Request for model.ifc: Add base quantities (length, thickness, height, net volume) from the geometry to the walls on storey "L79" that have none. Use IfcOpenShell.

First a look at what the model holds.

```python
import ifcopenshell
import ifcopenshell.util.element
import ifcopenshell.util.unit

model = ifcopenshell.open("model.ifc")
print(model.schema)
for unit_type in ("LENGTHUNIT", "AREAUNIT", "VOLUMEUNIT"):
    print(unit_type, ifcopenshell.util.unit.calculate_unit_scale(model, unit_type))
storey = next(s for s in model.by_type("IfcBuildingStorey") if s.Name == "L79")
walls = [e for e in ifcopenshell.util.element.get_decomposition(storey) if e.is_a("IfcWall")]
for e in sorted(walls, key=lambda e: e.id()):
    print(e.id(), e.is_a(), e.Name, list(ifcopenshell.util.element.get_psets(e, qtos_only=True)), sep=" | ")
```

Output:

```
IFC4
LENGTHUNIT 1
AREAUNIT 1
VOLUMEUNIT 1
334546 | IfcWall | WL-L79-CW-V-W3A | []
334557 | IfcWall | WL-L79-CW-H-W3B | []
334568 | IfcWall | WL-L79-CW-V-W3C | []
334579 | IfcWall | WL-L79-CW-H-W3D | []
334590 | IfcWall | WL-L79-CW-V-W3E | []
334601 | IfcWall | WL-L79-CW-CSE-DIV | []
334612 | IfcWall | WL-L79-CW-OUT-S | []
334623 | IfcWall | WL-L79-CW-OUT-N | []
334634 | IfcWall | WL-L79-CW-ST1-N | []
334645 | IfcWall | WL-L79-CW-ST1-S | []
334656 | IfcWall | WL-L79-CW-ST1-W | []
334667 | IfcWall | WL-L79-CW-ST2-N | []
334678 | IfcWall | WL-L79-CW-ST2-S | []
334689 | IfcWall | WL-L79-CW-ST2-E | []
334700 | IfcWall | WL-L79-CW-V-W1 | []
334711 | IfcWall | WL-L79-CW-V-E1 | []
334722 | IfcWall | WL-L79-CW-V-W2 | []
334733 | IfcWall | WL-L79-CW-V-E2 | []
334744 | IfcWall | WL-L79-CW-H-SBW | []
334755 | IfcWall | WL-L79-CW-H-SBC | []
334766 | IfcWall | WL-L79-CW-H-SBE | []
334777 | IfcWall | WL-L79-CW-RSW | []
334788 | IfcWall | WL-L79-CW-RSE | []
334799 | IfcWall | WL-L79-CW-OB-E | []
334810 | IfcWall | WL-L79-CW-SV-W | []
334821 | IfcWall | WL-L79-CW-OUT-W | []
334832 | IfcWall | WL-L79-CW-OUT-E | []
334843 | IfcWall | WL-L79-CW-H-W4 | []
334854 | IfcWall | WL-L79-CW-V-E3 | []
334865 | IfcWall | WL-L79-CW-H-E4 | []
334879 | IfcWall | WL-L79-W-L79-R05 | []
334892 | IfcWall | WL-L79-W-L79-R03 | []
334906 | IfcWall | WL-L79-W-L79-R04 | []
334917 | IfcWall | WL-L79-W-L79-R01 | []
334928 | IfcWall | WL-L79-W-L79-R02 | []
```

```python
import ifcopenshell
import ifcopenshell.api.pset
import ifcopenshell.geom
import ifcopenshell.util.element
import ifcopenshell.util.shape
import ifcopenshell.util.unit

model = ifcopenshell.open("model.ifc")
unit_scale = ifcopenshell.util.unit.calculate_unit_scale(model)
volume_scale = ifcopenshell.util.unit.calculate_unit_scale(model, "VOLUMEUNIT")
settings = ifcopenshell.geom.settings()

storey = next(s for s in model.by_type("IfcBuildingStorey") if s.Name == "L79")
walls = [e for e in ifcopenshell.util.element.get_decomposition(storey) if e.is_a("IfcWall")]

for e in sorted(walls, key=lambda e: e.id()):
    if ifcopenshell.util.element.get_psets(e, qtos_only=True, should_inherit=False):
        continue
    # Geometry comes back in metres, in the element's own axes.
    shape = ifcopenshell.geom.create_shape(settings, e)
    values = {
        "Length": ifcopenshell.util.shape.get_x(shape.geometry) / unit_scale,
        "Width": ifcopenshell.util.shape.get_y(shape.geometry) / unit_scale,
        "Height": ifcopenshell.util.shape.get_z(shape.geometry) / unit_scale,
        "NetVolume": ifcopenshell.util.shape.get_volume(shape.geometry) / volume_scale,
    }
    qto = ifcopenshell.api.pset.add_qto(model, product=e, name="Qto_WallBaseQuantities")
    ifcopenshell.api.pset.edit_qto(model, qto=qto, properties=values)
    print(e.id(), {k: round(v, 3) for k, v in values.items()})

model.write("model_rev.ifc")
```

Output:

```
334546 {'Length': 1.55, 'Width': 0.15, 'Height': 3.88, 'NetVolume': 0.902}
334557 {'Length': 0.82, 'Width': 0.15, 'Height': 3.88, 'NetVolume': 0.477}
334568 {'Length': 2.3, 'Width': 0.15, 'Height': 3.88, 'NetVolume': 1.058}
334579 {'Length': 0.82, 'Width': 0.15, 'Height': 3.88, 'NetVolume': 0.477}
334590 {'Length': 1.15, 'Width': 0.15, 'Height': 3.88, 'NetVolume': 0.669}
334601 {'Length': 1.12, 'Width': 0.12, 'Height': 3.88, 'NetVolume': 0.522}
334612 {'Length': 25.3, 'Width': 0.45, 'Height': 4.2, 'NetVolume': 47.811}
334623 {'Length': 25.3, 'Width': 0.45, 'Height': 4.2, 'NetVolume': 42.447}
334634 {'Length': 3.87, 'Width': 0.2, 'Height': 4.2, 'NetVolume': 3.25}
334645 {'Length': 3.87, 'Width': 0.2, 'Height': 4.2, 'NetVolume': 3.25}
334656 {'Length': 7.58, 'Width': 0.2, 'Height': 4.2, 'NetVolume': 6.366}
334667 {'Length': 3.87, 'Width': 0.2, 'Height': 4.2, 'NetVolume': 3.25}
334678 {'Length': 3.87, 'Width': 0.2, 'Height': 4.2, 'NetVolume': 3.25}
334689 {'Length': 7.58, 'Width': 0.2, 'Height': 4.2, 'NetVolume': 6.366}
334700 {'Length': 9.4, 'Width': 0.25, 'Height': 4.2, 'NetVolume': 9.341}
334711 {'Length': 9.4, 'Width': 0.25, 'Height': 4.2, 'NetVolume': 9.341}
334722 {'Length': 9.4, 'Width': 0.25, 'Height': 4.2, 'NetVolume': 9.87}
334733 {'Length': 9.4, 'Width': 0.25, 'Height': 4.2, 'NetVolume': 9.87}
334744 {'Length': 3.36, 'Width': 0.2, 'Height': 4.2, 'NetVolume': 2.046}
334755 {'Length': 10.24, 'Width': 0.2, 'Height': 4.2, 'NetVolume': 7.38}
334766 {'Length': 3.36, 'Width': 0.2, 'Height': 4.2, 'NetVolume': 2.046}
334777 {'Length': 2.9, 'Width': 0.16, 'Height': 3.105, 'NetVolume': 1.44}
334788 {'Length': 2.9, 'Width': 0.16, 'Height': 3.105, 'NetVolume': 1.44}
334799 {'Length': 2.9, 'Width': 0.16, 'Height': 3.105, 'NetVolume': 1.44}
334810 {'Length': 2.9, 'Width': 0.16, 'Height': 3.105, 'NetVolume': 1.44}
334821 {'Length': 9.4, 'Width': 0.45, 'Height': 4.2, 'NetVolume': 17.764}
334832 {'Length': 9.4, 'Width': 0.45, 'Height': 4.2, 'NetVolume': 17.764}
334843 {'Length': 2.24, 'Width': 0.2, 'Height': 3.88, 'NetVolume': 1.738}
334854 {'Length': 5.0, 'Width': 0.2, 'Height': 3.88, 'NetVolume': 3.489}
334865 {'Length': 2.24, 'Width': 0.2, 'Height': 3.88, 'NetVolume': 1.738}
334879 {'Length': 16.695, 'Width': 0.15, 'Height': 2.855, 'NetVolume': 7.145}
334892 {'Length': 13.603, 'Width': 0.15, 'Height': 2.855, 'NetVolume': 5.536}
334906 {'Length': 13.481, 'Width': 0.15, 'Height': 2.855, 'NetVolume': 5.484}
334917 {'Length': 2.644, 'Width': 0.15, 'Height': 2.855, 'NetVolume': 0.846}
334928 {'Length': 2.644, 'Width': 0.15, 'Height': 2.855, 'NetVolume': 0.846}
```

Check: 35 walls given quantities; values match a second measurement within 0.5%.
